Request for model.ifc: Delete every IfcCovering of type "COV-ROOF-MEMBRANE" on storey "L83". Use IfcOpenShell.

First a look at what the model holds.

```python
import ifcopenshell
import ifcopenshell.util.element

model = ifcopenshell.open("model.ifc")
print(model.schema)
storey = next(s for s in model.by_type("IfcBuildingStorey") if s.Name == "L83")
coverings = [e for e in ifcopenshell.util.element.get_decomposition(storey) if e.is_a("IfcCovering")]
seen = {}
for e in coverings:
    element_type = ifcopenshell.util.element.get_type(e)
    name = element_type.Name if element_type not in (None, e) else None
    seen[name] = seen.get(name, 0) + 1
for name, count in sorted(seen.items(), key=str):
    print(count, "x", name)
```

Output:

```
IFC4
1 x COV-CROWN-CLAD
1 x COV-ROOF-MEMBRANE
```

```python
import ifcopenshell
import ifcopenshell.api.root
import ifcopenshell.util.element

model = ifcopenshell.open("model.ifc")

storey = next(s for s in model.by_type("IfcBuildingStorey") if s.Name == "L83")
coverings = [e for e in ifcopenshell.util.element.get_decomposition(storey) if e.is_a("IfcCovering")]
targets = [e for e in coverings if (t := ifcopenshell.util.element.get_type(e)) not in (None, e) and t.Name == "COV-ROOF-MEMBRANE"]

for e in targets:
    ifcopenshell.api.root.remove_product(model, product=e)
print(len(targets), "removed")

model.write("model_rev.ifc")
```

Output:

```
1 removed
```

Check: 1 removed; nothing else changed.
